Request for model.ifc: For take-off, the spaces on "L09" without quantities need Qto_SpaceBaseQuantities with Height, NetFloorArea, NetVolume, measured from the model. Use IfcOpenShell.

First a look at what the model holds.

```python
import ifcopenshell
import ifcopenshell.util.element
import ifcopenshell.util.unit

model = ifcopenshell.open("model.ifc")
print(model.schema)
for unit_type in ("LENGTHUNIT", "AREAUNIT", "VOLUMEUNIT"):
    print(unit_type, ifcopenshell.util.unit.calculate_unit_scale(model, unit_type))
storey = next(s for s in model.by_type("IfcBuildingStorey") if s.Name == "L09")
spaces = [e for e in ifcopenshell.util.element.get_decomposition(storey) if e.is_a("IfcSpace")]
for e in sorted(spaces, key=lambda e: e.id()):
    print(e.id(), e.is_a(), e.Name, list(ifcopenshell.util.element.get_psets(e, qtos_only=True)), sep=" | ")
```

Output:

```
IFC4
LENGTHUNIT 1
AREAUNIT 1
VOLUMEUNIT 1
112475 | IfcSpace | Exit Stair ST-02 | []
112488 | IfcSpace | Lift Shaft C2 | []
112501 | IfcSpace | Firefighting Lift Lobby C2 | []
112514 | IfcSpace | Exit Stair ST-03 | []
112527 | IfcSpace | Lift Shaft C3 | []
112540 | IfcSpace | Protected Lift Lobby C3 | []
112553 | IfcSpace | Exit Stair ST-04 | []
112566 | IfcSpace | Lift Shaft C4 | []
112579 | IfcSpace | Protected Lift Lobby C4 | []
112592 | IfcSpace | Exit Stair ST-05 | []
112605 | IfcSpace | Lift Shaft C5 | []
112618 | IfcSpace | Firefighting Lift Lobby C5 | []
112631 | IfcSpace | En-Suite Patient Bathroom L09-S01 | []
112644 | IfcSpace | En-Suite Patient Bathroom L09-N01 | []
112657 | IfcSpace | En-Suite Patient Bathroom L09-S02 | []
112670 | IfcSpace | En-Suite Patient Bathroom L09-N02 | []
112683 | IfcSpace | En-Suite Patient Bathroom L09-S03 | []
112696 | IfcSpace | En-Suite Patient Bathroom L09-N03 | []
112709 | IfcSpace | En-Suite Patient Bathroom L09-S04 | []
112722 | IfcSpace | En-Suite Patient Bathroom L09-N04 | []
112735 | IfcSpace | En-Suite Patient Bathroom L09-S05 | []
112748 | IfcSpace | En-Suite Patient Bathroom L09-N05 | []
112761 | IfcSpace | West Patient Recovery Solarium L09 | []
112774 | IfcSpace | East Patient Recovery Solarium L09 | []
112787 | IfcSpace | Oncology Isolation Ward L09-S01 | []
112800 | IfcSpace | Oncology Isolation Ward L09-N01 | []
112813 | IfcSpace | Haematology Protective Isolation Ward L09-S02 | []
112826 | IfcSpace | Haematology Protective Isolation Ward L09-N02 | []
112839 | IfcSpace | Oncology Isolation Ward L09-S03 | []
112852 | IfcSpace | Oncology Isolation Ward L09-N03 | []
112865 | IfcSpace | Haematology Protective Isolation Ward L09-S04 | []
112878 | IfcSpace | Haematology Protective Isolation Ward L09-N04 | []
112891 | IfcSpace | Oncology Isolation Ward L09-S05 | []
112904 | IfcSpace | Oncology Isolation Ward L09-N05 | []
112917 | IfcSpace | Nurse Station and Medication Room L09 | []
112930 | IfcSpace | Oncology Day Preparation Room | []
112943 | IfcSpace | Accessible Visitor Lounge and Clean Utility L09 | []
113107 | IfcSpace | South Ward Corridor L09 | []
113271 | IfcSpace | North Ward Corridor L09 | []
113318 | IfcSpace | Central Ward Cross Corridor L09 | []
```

```python
import ifcopenshell
import ifcopenshell.api.pset
import ifcopenshell.geom
import ifcopenshell.util.element
import ifcopenshell.util.shape
import ifcopenshell.util.unit

model = ifcopenshell.open("model.ifc")
unit_scale = ifcopenshell.util.unit.calculate_unit_scale(model)
area_scale = ifcopenshell.util.unit.calculate_unit_scale(model, "AREAUNIT")
volume_scale = ifcopenshell.util.unit.calculate_unit_scale(model, "VOLUMEUNIT")
settings = ifcopenshell.geom.settings()

storey = next(s for s in model.by_type("IfcBuildingStorey") if s.Name == "L09")
spaces = [e for e in ifcopenshell.util.element.get_decomposition(storey) if e.is_a("IfcSpace")]

for e in sorted(spaces, key=lambda e: e.id()):
    if ifcopenshell.util.element.get_psets(e, qtos_only=True, should_inherit=False):
        continue
    # Geometry comes back in metres, in the element's own axes.
    shape = ifcopenshell.geom.create_shape(settings, e)
    values = {
        "Height": ifcopenshell.util.shape.get_z(shape.geometry) / unit_scale,
        "NetFloorArea": ifcopenshell.util.shape.get_footprint_area(shape.geometry) / area_scale,
        "NetVolume": ifcopenshell.util.shape.get_volume(shape.geometry) / volume_scale,
    }
    qto = ifcopenshell.api.pset.add_qto(model, product=e, name="Qto_SpaceBaseQuantities")
    ifcopenshell.api.pset.edit_qto(model, qto=qto, properties=values)
    print(e.id(), {k: round(v, 3) for k, v in values.items()})

model.write("model_updated.ifc")
```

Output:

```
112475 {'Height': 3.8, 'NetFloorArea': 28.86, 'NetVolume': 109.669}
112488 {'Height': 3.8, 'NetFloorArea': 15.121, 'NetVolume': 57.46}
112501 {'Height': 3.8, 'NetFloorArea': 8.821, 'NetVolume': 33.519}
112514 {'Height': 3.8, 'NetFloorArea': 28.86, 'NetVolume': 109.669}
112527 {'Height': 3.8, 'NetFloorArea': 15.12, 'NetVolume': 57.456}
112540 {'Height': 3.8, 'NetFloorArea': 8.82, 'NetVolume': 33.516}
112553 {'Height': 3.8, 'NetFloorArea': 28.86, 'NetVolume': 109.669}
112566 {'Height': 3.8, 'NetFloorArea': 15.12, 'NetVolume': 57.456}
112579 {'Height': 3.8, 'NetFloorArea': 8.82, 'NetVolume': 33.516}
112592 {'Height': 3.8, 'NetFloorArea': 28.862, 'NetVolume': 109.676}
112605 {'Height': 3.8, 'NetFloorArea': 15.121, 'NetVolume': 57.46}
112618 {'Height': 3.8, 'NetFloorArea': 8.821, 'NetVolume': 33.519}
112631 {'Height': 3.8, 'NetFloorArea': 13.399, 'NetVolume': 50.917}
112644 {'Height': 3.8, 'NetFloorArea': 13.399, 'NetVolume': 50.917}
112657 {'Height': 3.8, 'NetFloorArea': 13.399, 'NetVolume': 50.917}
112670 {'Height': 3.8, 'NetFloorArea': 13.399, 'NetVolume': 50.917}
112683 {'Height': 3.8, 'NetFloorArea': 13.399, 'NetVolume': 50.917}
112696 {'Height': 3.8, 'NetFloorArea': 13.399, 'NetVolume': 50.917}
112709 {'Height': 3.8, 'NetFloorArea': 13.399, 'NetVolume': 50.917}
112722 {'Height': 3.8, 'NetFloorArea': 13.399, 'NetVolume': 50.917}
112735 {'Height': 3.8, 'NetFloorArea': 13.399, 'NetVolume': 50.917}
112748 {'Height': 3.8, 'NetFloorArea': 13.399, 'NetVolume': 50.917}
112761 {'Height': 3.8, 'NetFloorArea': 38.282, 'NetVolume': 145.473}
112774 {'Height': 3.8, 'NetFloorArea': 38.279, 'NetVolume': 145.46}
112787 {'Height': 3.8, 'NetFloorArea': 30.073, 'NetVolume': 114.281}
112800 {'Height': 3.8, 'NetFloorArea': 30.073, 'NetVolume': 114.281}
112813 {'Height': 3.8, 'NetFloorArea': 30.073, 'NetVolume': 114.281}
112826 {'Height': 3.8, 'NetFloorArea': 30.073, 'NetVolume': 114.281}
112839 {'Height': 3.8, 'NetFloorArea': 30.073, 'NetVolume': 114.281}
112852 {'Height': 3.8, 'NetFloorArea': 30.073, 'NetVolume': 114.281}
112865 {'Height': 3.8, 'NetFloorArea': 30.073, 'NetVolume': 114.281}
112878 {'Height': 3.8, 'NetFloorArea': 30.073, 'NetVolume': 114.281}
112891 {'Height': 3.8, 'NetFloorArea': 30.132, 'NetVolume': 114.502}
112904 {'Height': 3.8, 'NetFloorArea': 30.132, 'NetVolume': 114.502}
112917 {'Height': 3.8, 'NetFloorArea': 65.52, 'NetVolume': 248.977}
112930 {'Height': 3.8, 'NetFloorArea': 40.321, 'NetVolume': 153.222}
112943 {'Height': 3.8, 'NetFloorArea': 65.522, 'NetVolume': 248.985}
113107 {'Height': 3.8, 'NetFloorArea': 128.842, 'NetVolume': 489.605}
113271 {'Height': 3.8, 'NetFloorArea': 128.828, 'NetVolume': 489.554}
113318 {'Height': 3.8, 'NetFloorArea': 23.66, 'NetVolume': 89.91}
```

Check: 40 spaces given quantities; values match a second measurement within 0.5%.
